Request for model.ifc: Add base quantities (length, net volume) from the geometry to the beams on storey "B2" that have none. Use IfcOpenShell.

First a look at what the model holds.

```python
import ifcopenshell
import ifcopenshell.util.element
import ifcopenshell.util.unit

model = ifcopenshell.open("model.ifc")
print(model.schema)
for unit_type in ("LENGTHUNIT", "AREAUNIT", "VOLUMEUNIT"):
    print(unit_type, ifcopenshell.util.unit.calculate_unit_scale(model, unit_type))
storey = next(s for s in model.by_type("IfcBuildingStorey") if s.Name == "B2")
beams = [e for e in ifcopenshell.util.element.get_decomposition(storey) if e.is_a("IfcBeam")]
for e in sorted(beams, key=lambda e: e.id()):
    print(e.id(), e.is_a(), e.Name, list(ifcopenshell.util.element.get_psets(e, qtos_only=True)), sep=" | ")
```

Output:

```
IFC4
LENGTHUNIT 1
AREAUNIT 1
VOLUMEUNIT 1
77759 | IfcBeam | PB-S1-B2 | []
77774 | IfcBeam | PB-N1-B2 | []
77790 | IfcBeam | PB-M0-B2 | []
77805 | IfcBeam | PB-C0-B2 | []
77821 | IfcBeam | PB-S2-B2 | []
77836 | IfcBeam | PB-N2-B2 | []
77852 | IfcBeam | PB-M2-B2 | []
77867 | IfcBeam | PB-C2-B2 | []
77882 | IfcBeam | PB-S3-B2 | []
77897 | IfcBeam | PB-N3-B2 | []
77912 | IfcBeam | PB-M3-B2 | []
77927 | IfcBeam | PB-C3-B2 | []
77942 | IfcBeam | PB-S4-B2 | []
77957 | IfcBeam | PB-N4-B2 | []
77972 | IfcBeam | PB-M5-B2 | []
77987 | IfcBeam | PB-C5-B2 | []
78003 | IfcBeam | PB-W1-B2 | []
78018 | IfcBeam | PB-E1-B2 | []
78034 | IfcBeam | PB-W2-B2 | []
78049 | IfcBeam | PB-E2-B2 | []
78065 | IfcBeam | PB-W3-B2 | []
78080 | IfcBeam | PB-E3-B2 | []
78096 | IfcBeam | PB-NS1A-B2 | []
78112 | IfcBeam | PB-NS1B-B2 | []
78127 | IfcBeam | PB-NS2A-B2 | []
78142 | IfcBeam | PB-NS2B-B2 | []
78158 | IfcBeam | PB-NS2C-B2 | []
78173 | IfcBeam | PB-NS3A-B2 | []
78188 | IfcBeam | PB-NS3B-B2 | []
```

```python
import ifcopenshell
import ifcopenshell.api.pset
import ifcopenshell.geom
import ifcopenshell.util.element
import ifcopenshell.util.shape
import ifcopenshell.util.unit

model = ifcopenshell.open("model.ifc")
unit_scale = ifcopenshell.util.unit.calculate_unit_scale(model)
volume_scale = ifcopenshell.util.unit.calculate_unit_scale(model, "VOLUMEUNIT")
settings = ifcopenshell.geom.settings()

storey = next(s for s in model.by_type("IfcBuildingStorey") if s.Name == "B2")
beams = [e for e in ifcopenshell.util.element.get_decomposition(storey) if e.is_a("IfcBeam")]

for e in sorted(beams, key=lambda e: e.id()):
    if ifcopenshell.util.element.get_psets(e, qtos_only=True, should_inherit=False):
        continue
    # Geometry comes back in metres, in the element's own axes.
    shape = ifcopenshell.geom.create_shape(settings, e)
    values = {
        "Length": ifcopenshell.util.shape.get_max_xyz(shape.geometry) / unit_scale,
        "NetVolume": ifcopenshell.util.shape.get_volume(shape.geometry) / volume_scale,
    }
    qto = ifcopenshell.api.pset.add_qto(model, product=e, name="Qto_BeamBaseQuantities")
    ifcopenshell.api.pset.edit_qto(model, qto=qto, properties=values)
    print(e.id(), {k: round(v, 3) for k, v in values.items()})

model.write("model_edited.ifc")
```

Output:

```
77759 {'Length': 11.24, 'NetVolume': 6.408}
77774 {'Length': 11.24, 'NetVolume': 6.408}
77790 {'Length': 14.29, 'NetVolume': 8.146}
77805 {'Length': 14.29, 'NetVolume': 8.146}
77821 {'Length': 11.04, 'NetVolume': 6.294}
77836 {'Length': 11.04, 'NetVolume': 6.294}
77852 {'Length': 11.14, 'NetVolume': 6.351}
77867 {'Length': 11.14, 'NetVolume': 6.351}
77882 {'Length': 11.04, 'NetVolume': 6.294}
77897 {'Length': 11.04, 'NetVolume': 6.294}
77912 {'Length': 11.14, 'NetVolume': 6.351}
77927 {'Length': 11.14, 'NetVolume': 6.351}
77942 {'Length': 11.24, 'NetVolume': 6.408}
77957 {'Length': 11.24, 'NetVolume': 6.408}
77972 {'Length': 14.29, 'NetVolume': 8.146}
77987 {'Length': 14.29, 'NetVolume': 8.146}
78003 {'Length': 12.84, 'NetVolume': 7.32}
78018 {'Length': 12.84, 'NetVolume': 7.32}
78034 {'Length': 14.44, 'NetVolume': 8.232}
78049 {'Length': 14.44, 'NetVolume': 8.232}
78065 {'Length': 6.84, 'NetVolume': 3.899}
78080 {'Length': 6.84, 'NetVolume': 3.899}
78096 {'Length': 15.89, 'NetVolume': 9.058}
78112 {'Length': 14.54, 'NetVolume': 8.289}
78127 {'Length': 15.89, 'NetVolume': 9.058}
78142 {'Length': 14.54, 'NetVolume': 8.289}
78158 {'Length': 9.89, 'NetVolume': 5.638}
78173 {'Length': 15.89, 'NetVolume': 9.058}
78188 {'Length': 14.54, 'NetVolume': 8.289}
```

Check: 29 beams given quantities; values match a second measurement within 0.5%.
